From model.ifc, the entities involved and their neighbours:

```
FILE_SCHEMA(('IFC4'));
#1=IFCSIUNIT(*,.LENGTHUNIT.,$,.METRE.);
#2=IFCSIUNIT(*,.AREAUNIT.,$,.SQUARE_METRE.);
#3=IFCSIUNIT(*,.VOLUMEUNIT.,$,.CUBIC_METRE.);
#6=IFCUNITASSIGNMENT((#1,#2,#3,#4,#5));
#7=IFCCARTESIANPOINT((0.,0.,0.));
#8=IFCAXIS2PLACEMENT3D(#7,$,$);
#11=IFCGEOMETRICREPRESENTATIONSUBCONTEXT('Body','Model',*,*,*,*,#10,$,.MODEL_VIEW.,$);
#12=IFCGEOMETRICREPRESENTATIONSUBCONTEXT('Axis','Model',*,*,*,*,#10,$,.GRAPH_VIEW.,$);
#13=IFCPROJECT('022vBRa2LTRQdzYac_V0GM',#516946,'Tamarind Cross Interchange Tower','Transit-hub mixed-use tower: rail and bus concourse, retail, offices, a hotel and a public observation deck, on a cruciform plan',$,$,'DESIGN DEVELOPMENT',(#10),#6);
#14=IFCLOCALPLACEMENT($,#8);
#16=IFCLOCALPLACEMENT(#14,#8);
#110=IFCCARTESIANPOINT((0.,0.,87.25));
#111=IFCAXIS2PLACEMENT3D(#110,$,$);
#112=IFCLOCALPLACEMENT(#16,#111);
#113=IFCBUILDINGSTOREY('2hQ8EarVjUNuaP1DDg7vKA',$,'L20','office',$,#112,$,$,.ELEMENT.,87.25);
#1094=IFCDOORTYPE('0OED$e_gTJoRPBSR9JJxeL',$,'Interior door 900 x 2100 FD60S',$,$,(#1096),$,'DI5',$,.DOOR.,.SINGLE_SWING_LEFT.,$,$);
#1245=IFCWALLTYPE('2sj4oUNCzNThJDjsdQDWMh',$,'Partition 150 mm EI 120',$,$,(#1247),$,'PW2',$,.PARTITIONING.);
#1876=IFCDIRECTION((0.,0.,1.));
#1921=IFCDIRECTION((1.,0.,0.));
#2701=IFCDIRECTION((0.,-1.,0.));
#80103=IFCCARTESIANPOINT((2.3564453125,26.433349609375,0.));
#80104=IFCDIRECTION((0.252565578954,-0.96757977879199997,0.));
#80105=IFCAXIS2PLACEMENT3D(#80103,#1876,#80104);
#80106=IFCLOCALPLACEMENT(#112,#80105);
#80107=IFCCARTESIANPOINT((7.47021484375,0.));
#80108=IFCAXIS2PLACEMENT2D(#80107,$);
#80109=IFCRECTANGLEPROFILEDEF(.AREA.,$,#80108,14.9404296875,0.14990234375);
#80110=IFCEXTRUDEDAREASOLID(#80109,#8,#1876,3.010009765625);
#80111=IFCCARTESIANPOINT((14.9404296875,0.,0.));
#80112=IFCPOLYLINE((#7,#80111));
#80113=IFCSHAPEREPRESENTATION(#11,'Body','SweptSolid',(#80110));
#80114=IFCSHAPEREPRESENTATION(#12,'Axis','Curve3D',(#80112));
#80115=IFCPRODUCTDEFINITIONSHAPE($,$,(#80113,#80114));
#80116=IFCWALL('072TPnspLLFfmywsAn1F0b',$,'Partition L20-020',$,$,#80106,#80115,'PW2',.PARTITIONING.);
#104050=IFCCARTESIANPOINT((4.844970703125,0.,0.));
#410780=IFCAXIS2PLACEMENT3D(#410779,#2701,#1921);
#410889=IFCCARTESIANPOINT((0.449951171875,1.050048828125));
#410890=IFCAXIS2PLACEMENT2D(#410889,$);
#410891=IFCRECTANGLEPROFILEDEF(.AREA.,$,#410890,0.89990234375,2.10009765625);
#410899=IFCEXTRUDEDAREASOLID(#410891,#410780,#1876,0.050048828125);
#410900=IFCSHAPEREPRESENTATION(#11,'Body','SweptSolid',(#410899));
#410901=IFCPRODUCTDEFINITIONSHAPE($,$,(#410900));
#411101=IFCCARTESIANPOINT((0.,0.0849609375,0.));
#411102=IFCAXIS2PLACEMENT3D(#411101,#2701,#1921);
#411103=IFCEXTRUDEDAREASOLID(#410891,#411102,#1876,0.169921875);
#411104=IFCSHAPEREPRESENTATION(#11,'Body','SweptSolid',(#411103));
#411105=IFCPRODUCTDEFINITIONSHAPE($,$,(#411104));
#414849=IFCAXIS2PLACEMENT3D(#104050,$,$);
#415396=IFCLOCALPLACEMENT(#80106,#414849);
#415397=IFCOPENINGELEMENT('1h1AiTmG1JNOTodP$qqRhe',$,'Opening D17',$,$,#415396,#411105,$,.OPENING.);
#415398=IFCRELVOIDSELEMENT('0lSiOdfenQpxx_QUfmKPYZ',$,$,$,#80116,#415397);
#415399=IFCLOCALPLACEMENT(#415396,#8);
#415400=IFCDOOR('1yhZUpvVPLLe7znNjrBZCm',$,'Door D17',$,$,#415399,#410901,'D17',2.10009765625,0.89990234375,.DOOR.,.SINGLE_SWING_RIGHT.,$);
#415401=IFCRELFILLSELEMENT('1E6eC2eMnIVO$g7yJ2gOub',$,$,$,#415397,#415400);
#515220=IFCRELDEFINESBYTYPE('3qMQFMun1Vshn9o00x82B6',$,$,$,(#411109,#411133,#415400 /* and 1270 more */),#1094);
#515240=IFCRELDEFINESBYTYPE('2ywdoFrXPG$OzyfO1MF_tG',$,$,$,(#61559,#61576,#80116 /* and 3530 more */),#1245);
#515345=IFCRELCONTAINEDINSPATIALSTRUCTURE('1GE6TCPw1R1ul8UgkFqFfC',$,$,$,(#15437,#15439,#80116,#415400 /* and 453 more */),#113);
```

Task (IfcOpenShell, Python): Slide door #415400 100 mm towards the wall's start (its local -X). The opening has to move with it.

```python
import ifcopenshell
import ifcopenshell.api.geometry
import ifcopenshell.util.placement

model = ifcopenshell.open("model.ifc")

door = model.by_guid("1yhZUpvVPLLe7znNjrBZCm")
opening = door.FillsVoids[0].RelatingOpeningElement
wall = opening.VoidsElements[0].RelatingBuildingElement

wall_matrix = ifcopenshell.util.placement.get_local_placement(wall.ObjectPlacement)
shift = wall_matrix[:3, 0] * -0.1
before = ifcopenshell.util.placement.get_local_placement(door.ObjectPlacement)[:3, 3].copy()

# The door is placed relative to its opening, so it follows when the opening moves.
matrix = ifcopenshell.util.placement.get_local_placement(opening.ObjectPlacement)
matrix[:3, 3] += shift
ifcopenshell.api.geometry.edit_object_placement(
    model, product=opening, matrix=matrix, is_si=False, should_transform_children=True
)

after = ifcopenshell.util.placement.get_local_placement(door.ObjectPlacement)[:3, 3]
print("door moved by", (after - before).round(3) + 0.0)

model.write("model_rev.ifc")
```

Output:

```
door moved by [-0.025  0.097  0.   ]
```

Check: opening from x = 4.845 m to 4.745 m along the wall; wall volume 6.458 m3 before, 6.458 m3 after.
